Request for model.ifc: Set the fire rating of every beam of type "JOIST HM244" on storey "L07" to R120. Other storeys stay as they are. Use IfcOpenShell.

First a look at what the model holds.

```python
import ifcopenshell
import ifcopenshell.util.element

model = ifcopenshell.open("model.ifc")
print(model.schema)
storey = next(s for s in model.by_type("IfcBuildingStorey") if s.Name == "L07")
beams = [e for e in ifcopenshell.util.element.get_decomposition(storey) if e.is_a("IfcBeam")]
seen = {}
for e in beams:
    element_type = ifcopenshell.util.element.get_type(e)
    key = (element_type.Name if element_type != e and element_type else None, ifcopenshell.util.element.get_pset(e, "Pset_BeamCommon", "FireRating"))
    seen[key] = seen.get(key, 0) + 1
for (name, value), count in sorted(seen.items(), key=str):
    print(count, "x", name, "|", value)
```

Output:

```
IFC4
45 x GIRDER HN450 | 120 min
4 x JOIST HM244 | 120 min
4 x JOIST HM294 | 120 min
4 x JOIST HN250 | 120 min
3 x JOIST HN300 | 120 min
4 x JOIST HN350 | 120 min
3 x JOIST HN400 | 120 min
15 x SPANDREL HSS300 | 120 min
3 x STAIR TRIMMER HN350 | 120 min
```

```python
import ifcopenshell
import ifcopenshell.api.pset
import ifcopenshell.util.element

model = ifcopenshell.open("model.ifc")

storey = next(s for s in model.by_type("IfcBuildingStorey") if s.Name == "L07")
beams = [e for e in ifcopenshell.util.element.get_decomposition(storey) if e.is_a("IfcBeam")]

count = 0
for e in beams:
    element_type = ifcopenshell.util.element.get_type(e)
    if element_type in (None, e) or element_type.Name != "JOIST HM244":
        continue
    # add_pset returns the element's existing set when there is one.
    pset = ifcopenshell.api.pset.add_pset(model, product=e, name="Pset_BeamCommon")
    ifcopenshell.api.pset.edit_pset(model, pset=pset, properties={"FireRating": "R120"})
    count += 1

print(count, "beams updated")

model.write("model_updated.ifc")
```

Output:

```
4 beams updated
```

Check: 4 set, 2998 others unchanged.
